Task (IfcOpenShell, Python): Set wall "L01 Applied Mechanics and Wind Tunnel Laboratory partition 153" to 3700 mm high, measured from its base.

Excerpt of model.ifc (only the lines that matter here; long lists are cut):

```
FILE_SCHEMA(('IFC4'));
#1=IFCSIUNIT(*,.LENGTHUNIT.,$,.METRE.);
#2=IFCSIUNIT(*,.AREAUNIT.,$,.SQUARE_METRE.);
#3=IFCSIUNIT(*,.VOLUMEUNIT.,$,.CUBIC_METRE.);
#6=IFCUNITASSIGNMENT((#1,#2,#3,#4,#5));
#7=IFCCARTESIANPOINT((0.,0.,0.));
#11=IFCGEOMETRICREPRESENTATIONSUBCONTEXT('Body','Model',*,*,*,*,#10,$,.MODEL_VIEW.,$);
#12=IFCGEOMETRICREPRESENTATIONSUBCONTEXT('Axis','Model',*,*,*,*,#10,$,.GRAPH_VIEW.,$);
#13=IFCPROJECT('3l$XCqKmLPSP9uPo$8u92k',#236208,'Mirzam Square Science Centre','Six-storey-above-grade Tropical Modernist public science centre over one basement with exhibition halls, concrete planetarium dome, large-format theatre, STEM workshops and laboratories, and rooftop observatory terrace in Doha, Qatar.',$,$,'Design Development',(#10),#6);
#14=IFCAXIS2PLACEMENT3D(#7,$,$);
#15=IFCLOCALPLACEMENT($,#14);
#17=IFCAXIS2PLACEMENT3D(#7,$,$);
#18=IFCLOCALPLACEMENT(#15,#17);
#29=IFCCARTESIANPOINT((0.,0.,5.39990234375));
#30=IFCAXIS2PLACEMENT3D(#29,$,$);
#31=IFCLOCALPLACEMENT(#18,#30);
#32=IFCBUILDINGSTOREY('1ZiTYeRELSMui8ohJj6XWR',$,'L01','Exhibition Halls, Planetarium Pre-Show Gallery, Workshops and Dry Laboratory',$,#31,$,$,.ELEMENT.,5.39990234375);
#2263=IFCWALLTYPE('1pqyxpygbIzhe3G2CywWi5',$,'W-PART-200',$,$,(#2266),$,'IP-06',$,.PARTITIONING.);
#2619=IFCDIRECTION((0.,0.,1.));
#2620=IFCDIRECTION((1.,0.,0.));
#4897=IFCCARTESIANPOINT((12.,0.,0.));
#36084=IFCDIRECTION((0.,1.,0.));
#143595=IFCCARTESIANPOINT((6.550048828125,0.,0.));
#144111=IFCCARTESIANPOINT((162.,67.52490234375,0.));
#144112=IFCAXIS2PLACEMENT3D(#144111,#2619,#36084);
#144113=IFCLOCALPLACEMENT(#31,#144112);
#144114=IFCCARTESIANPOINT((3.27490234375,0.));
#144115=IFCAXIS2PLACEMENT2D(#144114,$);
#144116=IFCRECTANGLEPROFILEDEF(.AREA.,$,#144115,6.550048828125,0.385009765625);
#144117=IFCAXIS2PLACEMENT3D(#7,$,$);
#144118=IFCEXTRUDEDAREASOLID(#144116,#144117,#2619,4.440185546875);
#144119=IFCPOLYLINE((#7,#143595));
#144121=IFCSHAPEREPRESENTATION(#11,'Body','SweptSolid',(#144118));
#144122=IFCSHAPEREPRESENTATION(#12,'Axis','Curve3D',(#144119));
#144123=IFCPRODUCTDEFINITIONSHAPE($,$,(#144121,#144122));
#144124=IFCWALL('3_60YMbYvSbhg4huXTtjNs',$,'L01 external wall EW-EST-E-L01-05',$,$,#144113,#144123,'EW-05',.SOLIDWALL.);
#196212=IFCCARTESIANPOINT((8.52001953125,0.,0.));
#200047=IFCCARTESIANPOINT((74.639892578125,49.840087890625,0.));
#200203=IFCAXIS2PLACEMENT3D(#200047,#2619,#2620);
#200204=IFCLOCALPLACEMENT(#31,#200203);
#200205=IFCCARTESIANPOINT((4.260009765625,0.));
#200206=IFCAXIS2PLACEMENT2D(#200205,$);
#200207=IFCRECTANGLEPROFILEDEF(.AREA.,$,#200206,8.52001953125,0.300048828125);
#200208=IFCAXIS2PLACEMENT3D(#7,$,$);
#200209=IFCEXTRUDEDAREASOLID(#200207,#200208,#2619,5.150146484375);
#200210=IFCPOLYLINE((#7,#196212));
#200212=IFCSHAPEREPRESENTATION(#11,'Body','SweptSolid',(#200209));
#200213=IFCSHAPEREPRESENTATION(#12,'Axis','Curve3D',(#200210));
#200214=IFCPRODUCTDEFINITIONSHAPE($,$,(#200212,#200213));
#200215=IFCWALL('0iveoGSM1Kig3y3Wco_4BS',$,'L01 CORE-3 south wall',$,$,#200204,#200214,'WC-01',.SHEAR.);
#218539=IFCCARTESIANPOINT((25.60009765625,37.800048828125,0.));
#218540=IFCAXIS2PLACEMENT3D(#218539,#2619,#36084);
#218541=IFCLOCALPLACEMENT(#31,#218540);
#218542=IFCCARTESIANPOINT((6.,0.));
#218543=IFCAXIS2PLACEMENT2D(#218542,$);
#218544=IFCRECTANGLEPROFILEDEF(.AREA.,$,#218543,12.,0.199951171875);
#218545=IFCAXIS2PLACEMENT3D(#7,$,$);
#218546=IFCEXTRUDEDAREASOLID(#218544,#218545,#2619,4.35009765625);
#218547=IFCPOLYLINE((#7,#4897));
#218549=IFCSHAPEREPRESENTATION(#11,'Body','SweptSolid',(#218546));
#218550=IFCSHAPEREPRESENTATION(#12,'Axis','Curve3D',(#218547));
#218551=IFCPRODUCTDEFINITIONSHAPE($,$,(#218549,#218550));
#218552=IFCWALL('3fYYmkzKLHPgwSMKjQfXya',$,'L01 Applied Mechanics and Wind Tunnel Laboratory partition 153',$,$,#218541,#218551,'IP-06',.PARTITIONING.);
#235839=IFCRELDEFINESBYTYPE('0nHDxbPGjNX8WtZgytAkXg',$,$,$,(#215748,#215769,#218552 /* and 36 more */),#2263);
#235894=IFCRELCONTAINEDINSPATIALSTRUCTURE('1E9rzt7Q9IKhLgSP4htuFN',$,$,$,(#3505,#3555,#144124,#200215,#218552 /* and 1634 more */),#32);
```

```python
import ifcopenshell
import ifcopenshell.geom
import ifcopenshell.util.representation
import ifcopenshell.util.shape

model = ifcopenshell.open("model.ifc")
settings = ifcopenshell.geom.settings()


def volume(element):
    """Net volume in cubic metres, openings subtracted."""
    shape = ifcopenshell.geom.create_shape(settings, element)
    return ifcopenshell.util.shape.get_volume(shape.geometry)


wall = model.by_guid("3fYYmkzKLHPgwSMKjQfXya")
before = volume(wall)

body = ifcopenshell.util.representation.get_representation(wall, "Model", "Body")
solid = body.Items[0]
old_height = solid.Depth
solid.Depth = 3.7
after = volume(wall)

print(f"height {old_height:g} -> {solid.Depth:g}, volume {before:.3f} -> {after:.3f} m3")

model.write("model_edited.ifc")
```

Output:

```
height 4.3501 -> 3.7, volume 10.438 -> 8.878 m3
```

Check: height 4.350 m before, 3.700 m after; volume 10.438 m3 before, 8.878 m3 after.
